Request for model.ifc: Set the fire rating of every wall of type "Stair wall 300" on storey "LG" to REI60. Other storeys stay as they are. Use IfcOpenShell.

First a look at what the model holds.

```python
import ifcopenshell
import ifcopenshell.util.element

model = ifcopenshell.open("model.ifc")
print(model.schema)
storey = next(s for s in model.by_type("IfcBuildingStorey") if s.Name == "LG")
walls = [e for e in ifcopenshell.util.element.get_decomposition(storey) if e.is_a("IfcWall")]
seen = {}
for e in walls:
    element_type = ifcopenshell.util.element.get_type(e)
    key = (element_type.Name if element_type != e and element_type else None, ifcopenshell.util.element.get_pset(e, "Pset_WallCommon", "FireRating"))
    seen[key] = seen.get(key, 0) + 1
for (name, value), count in sorted(seen.items(), key=str):
    print(count, "x", name, "|", value)
```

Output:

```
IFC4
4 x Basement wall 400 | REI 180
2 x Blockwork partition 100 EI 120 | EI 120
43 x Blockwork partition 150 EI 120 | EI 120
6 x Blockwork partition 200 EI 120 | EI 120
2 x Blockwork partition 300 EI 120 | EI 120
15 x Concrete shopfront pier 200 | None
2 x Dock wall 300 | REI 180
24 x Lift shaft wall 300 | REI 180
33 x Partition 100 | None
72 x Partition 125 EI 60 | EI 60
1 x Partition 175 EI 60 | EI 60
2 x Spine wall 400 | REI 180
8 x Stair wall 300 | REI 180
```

```python
import ifcopenshell
import ifcopenshell.api.pset
import ifcopenshell.util.element

model = ifcopenshell.open("model.ifc")

storey = next(s for s in model.by_type("IfcBuildingStorey") if s.Name == "LG")
walls = [e for e in ifcopenshell.util.element.get_decomposition(storey) if e.is_a("IfcWall")]

count = 0
for e in walls:
    element_type = ifcopenshell.util.element.get_type(e)
    if element_type in (None, e) or element_type.Name != "Stair wall 300":
        continue
    # add_pset returns the element's existing set when there is one.
    pset = ifcopenshell.api.pset.add_pset(model, product=e, name="Pset_WallCommon")
    ifcopenshell.api.pset.edit_pset(model, pset=pset, properties={"FireRating": "REI60"})
    count += 1

print(count, "walls updated")

model.write("model_updated.ifc")
```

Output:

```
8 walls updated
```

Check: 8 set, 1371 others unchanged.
